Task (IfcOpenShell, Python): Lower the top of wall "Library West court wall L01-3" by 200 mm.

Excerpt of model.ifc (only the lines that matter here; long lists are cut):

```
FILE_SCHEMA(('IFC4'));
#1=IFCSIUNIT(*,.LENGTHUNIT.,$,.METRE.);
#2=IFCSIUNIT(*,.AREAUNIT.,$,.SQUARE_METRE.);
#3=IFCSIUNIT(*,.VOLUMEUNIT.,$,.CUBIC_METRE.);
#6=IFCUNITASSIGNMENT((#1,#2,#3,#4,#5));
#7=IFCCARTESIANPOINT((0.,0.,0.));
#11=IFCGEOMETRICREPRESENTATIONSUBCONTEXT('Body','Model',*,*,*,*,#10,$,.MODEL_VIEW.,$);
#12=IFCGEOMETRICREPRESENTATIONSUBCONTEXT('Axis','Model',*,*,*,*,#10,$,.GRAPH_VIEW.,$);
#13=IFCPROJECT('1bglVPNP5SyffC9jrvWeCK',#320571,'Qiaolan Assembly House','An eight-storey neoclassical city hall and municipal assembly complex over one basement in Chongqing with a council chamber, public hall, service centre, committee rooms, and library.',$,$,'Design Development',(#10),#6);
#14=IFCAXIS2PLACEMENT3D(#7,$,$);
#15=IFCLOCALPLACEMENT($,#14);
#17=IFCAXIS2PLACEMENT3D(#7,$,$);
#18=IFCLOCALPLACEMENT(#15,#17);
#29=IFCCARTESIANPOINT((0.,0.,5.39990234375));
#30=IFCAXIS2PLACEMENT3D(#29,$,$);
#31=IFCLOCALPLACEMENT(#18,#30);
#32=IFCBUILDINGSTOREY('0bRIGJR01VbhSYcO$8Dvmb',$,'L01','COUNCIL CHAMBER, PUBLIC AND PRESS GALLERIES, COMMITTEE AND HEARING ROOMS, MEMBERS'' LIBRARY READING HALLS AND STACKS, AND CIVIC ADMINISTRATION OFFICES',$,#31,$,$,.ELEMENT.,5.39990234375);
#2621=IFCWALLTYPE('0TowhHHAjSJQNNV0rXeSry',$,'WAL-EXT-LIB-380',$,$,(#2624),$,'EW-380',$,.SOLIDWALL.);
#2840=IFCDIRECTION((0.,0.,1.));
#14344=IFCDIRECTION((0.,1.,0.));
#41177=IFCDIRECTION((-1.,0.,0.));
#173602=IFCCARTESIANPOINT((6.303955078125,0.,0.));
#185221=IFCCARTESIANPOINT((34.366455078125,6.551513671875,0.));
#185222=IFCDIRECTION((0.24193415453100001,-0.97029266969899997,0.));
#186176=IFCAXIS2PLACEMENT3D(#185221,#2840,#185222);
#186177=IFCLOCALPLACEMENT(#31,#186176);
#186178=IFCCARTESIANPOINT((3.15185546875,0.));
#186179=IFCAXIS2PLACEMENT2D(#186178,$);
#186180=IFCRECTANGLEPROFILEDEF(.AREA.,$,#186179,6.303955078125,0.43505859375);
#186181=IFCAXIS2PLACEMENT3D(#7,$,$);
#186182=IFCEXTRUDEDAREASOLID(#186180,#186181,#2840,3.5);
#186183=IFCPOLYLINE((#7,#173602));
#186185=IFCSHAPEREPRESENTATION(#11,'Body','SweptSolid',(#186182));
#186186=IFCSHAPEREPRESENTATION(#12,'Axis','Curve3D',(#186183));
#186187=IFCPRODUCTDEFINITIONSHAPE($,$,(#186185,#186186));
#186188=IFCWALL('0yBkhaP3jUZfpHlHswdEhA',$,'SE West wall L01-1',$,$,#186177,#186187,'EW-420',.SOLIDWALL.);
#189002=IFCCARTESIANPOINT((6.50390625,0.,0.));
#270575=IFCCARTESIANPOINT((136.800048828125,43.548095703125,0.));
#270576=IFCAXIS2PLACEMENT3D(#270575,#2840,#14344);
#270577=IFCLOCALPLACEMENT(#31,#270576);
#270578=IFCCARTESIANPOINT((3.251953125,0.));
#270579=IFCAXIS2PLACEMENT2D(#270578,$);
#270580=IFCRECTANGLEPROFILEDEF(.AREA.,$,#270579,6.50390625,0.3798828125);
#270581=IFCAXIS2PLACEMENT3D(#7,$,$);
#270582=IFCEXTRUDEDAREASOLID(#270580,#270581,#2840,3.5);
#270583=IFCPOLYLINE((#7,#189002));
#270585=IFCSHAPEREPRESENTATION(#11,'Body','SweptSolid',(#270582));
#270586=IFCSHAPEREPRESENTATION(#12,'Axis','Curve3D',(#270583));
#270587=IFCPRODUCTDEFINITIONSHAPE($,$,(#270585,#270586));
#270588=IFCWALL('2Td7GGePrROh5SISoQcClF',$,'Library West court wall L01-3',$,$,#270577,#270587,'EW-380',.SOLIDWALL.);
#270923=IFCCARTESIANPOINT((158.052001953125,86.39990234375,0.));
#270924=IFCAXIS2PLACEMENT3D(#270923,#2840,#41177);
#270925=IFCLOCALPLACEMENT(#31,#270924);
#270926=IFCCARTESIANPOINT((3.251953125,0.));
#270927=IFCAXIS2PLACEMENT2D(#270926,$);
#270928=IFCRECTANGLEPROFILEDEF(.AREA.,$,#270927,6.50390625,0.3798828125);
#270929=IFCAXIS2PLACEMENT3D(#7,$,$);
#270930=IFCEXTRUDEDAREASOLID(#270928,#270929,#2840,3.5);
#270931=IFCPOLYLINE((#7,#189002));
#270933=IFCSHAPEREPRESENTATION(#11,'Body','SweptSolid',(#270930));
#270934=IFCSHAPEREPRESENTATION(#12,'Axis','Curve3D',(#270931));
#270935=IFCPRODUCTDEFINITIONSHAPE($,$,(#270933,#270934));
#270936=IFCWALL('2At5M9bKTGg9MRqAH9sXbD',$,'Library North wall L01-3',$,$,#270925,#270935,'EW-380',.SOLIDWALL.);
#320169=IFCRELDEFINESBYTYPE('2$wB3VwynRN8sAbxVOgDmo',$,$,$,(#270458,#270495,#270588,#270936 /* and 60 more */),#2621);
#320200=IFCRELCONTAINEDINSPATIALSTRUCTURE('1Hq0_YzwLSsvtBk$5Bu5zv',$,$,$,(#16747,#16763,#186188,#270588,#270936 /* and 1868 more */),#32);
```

```python
import ifcopenshell
import ifcopenshell.geom
import ifcopenshell.util.representation
import ifcopenshell.util.shape

model = ifcopenshell.open("model.ifc")
settings = ifcopenshell.geom.settings()


def volume(element):
    """Net volume in cubic metres, openings subtracted."""
    shape = ifcopenshell.geom.create_shape(settings, element)
    return ifcopenshell.util.shape.get_volume(shape.geometry)


wall = model.by_id(270588)
before = volume(wall)

body = ifcopenshell.util.representation.get_representation(wall, "Model", "Body")
solid = body.Items[0]
old_height = solid.Depth
solid.Depth -= 0.2
after = volume(wall)

print(f"height {old_height:g} -> {solid.Depth:g}, volume {before:.3f} -> {after:.3f} m3")

model.write("model_edited.ifc")
```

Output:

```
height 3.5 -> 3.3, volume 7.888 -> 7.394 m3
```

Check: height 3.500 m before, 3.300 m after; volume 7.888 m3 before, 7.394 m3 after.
